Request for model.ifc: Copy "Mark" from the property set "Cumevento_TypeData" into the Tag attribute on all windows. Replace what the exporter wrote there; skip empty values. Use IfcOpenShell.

First a look at what the model holds.

```python
import ifcopenshell
import ifcopenshell.util.element

model = ifcopenshell.open("model.ifc")
print(model.schema)
windows = model.by_type("IfcWindow")
print(len(windows), "windows")
for e in windows[:8]:
    source = ifcopenshell.util.element.get_pset(e, "Cumevento_TypeData", "Mark")
    target = e.Tag
    print(e.id(), repr(source), repr(target), sep=" | ")
```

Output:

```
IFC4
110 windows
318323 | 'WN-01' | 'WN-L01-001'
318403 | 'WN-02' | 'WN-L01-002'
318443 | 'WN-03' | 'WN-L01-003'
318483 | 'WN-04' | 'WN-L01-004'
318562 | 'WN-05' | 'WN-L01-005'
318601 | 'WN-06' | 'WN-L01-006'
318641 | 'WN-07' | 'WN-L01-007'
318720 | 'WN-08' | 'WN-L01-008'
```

```python
import ifcopenshell
import ifcopenshell.util.element

model = ifcopenshell.open("model.ifc")

count = 0
for e in model.by_type("IfcWindow"):
    value = ifcopenshell.util.element.get_pset(e, "Cumevento_TypeData", "Mark")
    current = e.Tag
    if not value or not value.strip() or current == value:
        continue
    e.Tag = value
    count += 1

print(count, "windows updated")

model.write("model_updated.ifc")
```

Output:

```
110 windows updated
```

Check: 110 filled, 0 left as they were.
